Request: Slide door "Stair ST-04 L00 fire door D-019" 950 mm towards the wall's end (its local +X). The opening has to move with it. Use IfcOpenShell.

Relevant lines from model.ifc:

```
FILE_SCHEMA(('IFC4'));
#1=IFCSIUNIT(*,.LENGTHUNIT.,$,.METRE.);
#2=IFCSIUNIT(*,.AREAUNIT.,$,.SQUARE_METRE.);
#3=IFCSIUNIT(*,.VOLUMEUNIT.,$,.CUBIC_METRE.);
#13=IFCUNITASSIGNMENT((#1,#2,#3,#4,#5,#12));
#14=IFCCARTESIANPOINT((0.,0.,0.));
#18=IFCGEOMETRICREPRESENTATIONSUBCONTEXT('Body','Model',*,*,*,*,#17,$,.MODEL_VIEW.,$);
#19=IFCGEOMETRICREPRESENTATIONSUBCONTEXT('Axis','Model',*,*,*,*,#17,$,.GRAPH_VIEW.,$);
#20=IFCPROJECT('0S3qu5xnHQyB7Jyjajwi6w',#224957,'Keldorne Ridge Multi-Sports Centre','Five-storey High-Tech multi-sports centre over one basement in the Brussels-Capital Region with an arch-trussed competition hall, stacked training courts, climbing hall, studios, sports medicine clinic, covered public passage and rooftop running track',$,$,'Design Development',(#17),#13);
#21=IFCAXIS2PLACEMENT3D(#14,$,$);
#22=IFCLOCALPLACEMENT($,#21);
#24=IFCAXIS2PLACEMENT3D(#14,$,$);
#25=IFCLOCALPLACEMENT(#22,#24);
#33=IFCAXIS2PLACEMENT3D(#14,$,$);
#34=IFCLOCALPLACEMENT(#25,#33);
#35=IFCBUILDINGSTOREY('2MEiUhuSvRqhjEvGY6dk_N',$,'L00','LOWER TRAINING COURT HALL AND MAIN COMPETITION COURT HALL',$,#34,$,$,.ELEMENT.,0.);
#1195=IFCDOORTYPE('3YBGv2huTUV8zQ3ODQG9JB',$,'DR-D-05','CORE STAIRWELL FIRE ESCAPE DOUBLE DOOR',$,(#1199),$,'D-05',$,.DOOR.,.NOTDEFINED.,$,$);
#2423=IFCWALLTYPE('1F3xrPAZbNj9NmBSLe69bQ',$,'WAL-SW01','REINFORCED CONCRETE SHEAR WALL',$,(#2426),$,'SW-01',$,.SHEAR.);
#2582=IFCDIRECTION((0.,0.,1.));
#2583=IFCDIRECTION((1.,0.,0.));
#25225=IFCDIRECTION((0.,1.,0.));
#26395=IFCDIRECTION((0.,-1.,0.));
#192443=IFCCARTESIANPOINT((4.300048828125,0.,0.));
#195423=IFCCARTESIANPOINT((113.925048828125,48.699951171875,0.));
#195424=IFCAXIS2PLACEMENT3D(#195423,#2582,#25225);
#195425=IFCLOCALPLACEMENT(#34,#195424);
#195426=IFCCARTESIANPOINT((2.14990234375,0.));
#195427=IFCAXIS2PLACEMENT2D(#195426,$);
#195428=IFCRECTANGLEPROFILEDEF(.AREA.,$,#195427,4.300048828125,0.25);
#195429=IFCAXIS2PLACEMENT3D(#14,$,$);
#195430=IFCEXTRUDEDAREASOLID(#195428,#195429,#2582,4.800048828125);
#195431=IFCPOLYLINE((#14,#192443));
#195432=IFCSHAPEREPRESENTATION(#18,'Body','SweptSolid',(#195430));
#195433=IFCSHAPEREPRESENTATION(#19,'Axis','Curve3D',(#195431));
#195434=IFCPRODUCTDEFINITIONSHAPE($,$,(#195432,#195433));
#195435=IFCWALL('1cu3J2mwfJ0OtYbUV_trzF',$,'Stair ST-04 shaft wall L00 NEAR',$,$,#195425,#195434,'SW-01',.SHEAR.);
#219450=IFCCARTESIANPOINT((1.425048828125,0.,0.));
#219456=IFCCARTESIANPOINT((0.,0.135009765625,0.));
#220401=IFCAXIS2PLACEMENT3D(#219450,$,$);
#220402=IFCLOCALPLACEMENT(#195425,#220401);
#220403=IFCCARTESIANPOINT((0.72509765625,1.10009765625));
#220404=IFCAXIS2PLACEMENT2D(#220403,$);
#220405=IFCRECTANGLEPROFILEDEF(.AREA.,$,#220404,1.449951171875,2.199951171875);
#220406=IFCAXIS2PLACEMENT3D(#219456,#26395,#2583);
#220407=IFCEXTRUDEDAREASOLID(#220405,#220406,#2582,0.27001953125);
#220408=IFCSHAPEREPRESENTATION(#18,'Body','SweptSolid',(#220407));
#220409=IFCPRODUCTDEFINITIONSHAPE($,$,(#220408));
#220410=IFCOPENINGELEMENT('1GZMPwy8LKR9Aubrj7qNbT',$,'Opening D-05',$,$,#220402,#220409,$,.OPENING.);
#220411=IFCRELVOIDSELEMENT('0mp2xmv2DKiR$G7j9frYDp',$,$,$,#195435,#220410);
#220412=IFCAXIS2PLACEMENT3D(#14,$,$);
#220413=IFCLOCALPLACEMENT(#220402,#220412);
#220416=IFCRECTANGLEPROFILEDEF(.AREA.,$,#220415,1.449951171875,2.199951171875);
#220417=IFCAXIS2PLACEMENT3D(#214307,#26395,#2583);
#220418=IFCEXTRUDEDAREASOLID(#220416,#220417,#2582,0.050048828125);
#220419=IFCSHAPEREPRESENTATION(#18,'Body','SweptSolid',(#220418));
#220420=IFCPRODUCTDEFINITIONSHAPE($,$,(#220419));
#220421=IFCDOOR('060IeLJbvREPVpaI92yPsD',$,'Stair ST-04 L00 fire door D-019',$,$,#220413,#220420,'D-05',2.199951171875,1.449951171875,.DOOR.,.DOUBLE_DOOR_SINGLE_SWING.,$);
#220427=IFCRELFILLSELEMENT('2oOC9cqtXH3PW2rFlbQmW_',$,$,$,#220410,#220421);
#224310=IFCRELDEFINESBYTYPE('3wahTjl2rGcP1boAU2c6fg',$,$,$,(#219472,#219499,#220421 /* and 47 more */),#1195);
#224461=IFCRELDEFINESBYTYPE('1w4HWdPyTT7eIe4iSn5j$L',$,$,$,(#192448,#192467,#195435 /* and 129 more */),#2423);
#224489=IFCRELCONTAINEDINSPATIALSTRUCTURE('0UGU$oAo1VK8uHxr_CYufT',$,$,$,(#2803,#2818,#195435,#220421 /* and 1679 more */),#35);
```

```python
import ifcopenshell
import ifcopenshell.api.geometry
import ifcopenshell.util.placement
import ifcopenshell.util.unit

model = ifcopenshell.open("model.ifc")
unit_scale = ifcopenshell.util.unit.calculate_unit_scale(model)

door = model.by_guid("060IeLJbvREPVpaI92yPsD")
opening = door.FillsVoids[0].RelatingOpeningElement
wall = opening.VoidsElements[0].RelatingBuildingElement

wall_matrix = ifcopenshell.util.placement.get_local_placement(wall.ObjectPlacement)
shift = wall_matrix[:3, 0] * 0.95 / unit_scale
before = ifcopenshell.util.placement.get_local_placement(door.ObjectPlacement)[:3, 3].copy()

# The door is placed relative to its opening, so it follows when the opening moves.
matrix = ifcopenshell.util.placement.get_local_placement(opening.ObjectPlacement)
matrix[:3, 3] += shift
ifcopenshell.api.geometry.edit_object_placement(
    model, product=opening, matrix=matrix, is_si=False, should_transform_children=True
)

after = ifcopenshell.util.placement.get_local_placement(door.ObjectPlacement)[:3, 3]
print("door moved by", (after - before).round(3) + 0.0)

model.write("model_updated.ifc")
```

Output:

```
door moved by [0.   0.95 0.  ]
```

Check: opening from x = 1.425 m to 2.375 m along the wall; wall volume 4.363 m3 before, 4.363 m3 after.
